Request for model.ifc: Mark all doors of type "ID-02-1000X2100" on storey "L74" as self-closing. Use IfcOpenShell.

First a look at what the model holds.

```python
import ifcopenshell
import ifcopenshell.util.element

model = ifcopenshell.open("model.ifc")
print(model.schema)
storey = next(s for s in model.by_type("IfcBuildingStorey") if s.Name == "L74")
doors = [e for e in ifcopenshell.util.element.get_decomposition(storey) if e.is_a("IfcDoor")]
seen = {}
for e in doors:
    element_type = ifcopenshell.util.element.get_type(e)
    key = (element_type.Name if element_type != e and element_type else None, ifcopenshell.util.element.get_pset(e, "Pset_DoorCommon", "SelfClosing"))
    seen[key] = seen.get(key, 0) + 1
for (name, value), count in sorted(seen.items(), key=str):
    print(count, "x", name, "|", value)
```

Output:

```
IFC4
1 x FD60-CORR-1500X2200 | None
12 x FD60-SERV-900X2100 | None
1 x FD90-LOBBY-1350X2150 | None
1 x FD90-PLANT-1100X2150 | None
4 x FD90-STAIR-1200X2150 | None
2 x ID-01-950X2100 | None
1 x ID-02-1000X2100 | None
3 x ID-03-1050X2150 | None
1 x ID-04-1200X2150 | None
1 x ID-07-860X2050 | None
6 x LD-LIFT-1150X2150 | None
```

```python
import ifcopenshell
import ifcopenshell.api.pset
import ifcopenshell.util.element

model = ifcopenshell.open("model.ifc")

storey = next(s for s in model.by_type("IfcBuildingStorey") if s.Name == "L74")
doors = [e for e in ifcopenshell.util.element.get_decomposition(storey) if e.is_a("IfcDoor")]

count = 0
for e in doors:
    element_type = ifcopenshell.util.element.get_type(e)
    if element_type in (None, e) or element_type.Name != "ID-02-1000X2100":
        continue
    # add_pset returns the element's existing set when there is one.
    pset = ifcopenshell.api.pset.add_pset(model, product=e, name="Pset_DoorCommon")
    ifcopenshell.api.pset.edit_pset(model, pset=pset, properties={"SelfClosing": True})
    count += 1

print(count, "doors updated")

model.write("model_updated.ifc")
```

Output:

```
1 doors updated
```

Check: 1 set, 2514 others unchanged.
